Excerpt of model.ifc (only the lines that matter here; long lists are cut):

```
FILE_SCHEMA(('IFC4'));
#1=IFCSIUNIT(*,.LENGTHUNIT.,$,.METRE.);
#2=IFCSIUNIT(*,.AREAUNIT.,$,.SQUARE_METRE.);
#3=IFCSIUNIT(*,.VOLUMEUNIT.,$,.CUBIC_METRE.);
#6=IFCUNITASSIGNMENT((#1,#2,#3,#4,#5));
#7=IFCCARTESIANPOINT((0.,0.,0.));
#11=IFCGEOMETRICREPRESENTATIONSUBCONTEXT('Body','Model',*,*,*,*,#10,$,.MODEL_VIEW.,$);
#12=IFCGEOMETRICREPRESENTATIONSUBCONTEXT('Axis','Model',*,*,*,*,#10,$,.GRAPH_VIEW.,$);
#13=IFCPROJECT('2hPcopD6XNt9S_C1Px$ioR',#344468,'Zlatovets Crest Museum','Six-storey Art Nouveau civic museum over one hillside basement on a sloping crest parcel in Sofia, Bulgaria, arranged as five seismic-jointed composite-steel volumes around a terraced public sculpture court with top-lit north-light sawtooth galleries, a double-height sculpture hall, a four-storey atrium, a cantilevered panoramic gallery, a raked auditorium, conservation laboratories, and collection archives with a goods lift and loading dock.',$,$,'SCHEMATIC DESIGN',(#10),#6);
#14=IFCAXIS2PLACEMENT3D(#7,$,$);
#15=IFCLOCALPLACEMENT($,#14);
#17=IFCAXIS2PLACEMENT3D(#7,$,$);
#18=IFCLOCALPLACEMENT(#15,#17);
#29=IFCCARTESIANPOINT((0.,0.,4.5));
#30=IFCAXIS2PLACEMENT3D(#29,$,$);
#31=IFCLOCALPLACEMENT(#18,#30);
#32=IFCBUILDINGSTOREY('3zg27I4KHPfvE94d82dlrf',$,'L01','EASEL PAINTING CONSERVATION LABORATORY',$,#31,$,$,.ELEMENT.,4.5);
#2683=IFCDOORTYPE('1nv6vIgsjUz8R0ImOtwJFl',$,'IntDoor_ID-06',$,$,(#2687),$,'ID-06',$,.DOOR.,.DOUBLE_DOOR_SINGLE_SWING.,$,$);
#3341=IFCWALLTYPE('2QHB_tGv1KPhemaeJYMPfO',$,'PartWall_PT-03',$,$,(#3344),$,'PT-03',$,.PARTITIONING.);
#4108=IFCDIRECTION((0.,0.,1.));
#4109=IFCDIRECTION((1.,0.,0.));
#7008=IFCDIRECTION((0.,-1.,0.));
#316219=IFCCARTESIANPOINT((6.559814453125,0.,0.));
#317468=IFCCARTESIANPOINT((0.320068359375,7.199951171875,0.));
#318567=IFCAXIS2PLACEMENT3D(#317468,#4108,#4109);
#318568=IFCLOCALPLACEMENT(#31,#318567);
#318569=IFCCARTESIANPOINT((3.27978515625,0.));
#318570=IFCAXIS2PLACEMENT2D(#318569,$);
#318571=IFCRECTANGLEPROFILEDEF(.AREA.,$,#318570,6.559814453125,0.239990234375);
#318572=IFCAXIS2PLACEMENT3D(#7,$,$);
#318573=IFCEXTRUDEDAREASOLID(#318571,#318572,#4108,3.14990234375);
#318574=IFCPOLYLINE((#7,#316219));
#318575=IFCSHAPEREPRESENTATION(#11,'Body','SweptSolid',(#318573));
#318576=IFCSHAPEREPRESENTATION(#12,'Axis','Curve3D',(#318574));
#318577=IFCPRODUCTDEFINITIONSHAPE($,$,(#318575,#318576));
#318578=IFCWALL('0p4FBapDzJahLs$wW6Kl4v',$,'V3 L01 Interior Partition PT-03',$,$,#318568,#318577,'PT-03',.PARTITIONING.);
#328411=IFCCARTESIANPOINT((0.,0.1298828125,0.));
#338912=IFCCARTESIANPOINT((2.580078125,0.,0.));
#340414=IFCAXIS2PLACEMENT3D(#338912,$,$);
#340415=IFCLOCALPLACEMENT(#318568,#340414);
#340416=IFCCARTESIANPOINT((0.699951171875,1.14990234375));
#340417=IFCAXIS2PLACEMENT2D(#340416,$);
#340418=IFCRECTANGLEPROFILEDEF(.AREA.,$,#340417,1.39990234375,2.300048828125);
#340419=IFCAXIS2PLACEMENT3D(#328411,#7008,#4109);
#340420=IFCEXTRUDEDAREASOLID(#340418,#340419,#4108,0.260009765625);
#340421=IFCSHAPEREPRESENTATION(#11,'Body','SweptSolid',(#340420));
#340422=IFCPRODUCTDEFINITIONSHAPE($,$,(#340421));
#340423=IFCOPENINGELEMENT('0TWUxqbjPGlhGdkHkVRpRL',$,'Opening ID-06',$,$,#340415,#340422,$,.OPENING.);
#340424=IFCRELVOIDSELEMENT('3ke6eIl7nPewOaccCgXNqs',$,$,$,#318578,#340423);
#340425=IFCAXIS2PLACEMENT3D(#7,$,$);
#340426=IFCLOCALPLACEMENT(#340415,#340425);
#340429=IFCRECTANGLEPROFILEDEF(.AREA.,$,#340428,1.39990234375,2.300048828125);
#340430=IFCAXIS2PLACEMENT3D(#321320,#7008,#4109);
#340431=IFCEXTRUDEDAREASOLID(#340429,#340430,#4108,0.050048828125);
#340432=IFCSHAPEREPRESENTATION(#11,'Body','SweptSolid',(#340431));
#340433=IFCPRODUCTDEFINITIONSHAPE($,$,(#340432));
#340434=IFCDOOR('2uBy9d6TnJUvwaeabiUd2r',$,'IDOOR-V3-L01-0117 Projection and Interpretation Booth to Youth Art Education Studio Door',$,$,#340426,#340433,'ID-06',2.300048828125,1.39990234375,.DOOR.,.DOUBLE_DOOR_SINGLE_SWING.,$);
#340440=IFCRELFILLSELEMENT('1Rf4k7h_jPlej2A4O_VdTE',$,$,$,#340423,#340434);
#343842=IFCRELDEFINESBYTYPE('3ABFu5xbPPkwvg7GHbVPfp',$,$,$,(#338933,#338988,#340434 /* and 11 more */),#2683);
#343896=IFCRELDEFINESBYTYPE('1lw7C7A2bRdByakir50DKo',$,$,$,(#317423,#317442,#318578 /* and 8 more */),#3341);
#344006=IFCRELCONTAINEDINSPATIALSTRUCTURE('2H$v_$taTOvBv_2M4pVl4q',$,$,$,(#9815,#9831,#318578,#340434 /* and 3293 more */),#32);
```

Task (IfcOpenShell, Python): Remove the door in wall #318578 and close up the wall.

```python
import ifcopenshell
import ifcopenshell.api.feature
import ifcopenshell.api.root
import ifcopenshell.geom
import ifcopenshell.util.shape

model = ifcopenshell.open("model.ifc")
settings = ifcopenshell.geom.settings()


def volume(element):
    """Net volume in cubic metres, openings subtracted."""
    shape = ifcopenshell.geom.create_shape(settings, element)
    return ifcopenshell.util.shape.get_volume(shape.geometry)


door = model.by_guid("2uBy9d6TnJUvwaeabiUd2r")
opening = door.FillsVoids[0].RelatingOpeningElement
wall = opening.VoidsElements[0].RelatingBuildingElement
before = volume(wall)

ifcopenshell.api.root.remove_product(model, product=door)
ifcopenshell.api.feature.remove_feature(model, feature=opening)

after = volume(wall)

print(f"wall volume {before:.3f} -> {after:.3f} m3")

model.write("model_v2.ifc")
```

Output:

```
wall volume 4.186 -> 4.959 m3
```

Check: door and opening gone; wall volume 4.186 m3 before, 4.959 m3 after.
